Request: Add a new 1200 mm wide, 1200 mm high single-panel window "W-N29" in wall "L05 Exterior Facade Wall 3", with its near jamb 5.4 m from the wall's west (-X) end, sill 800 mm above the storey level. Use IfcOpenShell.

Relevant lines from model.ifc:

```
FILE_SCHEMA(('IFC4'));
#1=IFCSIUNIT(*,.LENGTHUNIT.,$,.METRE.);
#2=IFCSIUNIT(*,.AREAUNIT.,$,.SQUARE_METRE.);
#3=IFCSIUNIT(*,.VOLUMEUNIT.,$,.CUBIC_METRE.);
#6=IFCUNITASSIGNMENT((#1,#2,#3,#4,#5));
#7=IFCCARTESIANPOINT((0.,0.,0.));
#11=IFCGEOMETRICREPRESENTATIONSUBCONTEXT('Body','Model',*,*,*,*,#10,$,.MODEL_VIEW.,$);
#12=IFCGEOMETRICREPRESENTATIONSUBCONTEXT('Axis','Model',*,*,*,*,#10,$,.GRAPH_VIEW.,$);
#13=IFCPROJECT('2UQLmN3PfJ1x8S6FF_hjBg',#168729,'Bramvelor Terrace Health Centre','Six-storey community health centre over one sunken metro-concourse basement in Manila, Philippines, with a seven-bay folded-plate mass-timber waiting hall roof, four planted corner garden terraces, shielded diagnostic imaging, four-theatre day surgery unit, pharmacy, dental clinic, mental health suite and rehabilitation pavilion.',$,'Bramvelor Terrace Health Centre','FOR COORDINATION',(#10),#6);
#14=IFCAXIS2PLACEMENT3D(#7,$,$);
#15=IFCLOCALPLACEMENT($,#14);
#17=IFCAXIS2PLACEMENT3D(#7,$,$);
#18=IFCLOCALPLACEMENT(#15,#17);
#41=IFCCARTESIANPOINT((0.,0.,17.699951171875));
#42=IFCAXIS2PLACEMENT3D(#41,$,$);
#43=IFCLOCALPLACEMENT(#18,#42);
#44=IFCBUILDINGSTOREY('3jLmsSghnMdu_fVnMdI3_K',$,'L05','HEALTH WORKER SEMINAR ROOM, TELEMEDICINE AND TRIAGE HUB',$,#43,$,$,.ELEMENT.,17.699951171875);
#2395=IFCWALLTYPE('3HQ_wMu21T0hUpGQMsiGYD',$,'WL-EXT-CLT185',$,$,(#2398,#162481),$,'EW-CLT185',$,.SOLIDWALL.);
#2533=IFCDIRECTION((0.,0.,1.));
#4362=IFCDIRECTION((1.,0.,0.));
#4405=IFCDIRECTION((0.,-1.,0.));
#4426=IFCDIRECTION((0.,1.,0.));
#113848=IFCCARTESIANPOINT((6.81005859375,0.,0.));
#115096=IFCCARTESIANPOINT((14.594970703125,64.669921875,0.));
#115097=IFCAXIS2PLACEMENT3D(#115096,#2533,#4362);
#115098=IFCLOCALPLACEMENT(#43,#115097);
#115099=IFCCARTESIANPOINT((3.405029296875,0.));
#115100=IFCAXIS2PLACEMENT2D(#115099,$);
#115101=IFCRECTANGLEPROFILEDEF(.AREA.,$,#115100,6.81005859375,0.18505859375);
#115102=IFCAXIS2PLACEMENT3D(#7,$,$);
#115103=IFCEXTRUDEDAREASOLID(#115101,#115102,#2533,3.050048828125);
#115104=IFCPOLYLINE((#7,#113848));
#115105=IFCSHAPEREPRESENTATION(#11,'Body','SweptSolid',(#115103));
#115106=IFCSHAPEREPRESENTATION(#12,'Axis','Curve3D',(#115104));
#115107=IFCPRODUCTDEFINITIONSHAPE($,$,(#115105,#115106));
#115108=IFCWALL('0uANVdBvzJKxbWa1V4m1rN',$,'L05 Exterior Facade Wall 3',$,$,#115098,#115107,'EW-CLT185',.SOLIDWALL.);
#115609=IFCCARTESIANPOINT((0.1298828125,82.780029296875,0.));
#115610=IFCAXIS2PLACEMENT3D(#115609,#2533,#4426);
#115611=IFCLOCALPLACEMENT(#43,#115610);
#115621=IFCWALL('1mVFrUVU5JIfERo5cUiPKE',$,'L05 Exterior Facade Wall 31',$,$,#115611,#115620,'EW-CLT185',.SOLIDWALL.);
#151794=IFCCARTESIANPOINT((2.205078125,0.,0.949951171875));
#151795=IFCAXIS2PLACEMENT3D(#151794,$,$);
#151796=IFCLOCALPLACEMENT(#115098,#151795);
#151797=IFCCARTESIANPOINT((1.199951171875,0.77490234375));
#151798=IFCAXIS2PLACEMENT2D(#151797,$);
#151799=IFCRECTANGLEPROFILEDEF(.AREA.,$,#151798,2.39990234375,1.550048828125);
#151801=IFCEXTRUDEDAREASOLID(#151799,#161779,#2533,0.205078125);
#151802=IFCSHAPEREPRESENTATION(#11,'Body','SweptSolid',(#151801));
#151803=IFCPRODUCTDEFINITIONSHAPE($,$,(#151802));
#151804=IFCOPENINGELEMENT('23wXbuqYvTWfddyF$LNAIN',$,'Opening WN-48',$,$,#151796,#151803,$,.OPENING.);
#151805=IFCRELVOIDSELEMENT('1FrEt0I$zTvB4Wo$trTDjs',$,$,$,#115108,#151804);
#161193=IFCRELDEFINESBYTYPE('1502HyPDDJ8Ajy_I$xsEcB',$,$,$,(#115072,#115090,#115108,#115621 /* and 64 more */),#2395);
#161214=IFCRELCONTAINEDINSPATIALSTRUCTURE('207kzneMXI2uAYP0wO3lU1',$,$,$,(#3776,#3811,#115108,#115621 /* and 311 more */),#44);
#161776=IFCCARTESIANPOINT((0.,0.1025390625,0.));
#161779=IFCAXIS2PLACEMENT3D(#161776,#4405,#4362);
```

```python
import numpy as np
import ifcopenshell
import ifcopenshell.api.feature
import ifcopenshell.api.geometry
import ifcopenshell.api.root
import ifcopenshell.api.spatial
import ifcopenshell.geom
import ifcopenshell.util.element
import ifcopenshell.util.placement
import ifcopenshell.util.representation
import ifcopenshell.util.shape
import ifcopenshell.util.unit

model = ifcopenshell.open("model.ifc")
unit_scale = ifcopenshell.util.unit.calculate_unit_scale(model)
settings = ifcopenshell.geom.settings()


def volume(element):
    """Net volume in cubic metres, openings subtracted."""
    shape = ifcopenshell.geom.create_shape(settings, element)
    return ifcopenshell.util.shape.get_volume(shape.geometry)


wall = model.by_guid("0uANVdBvzJKxbWa1V4m1rN")
storey = ifcopenshell.util.element.get_container(wall, ifc_class="IfcBuildingStorey")
context = ifcopenshell.util.representation.get_context(model, "Model", "Body", "MODEL_VIEW")
before = volume(wall)

width, height, from_end, sill = 1.2, 1.2, 5.4, 0.8  # metres

# The wall runs along its own X axis, and the end named is its -X end.
wall_shape = ifcopenshell.geom.create_shape(settings, wall)
x, y, z = ifcopenshell.util.shape.get_vertices(wall_shape.geometry).T
start = x.min() + from_end
face, thickness = float(y.min()), float(y.max() - y.min())
wall_matrix = ifcopenshell.util.placement.get_local_placement(wall.ObjectPlacement)
level = ifcopenshell.util.placement.get_local_placement(storey.ObjectPlacement)[2, 3]


def in_wall(x, y):
    """Placement at x, y metres in the wall's axes, at sill height."""
    matrix = wall_matrix.copy()
    matrix[:, 3] = wall_matrix @ np.array([x / unit_scale, y / unit_scale, 0.0, 1.0])
    matrix[2, 3] = level + sill / unit_scale
    return matrix


# Opening: a box that overshoots both wall faces by 50 mm.
opening = ifcopenshell.api.root.create_entity(model, ifc_class="IfcOpeningElement", predefined_type="OPENING")
box = ifcopenshell.api.geometry.add_wall_representation(
    model, context=context, length=width, height=height, thickness=thickness + 0.1
)
ifcopenshell.api.geometry.assign_representation(model, product=opening, representation=box)
ifcopenshell.api.geometry.edit_object_placement(model, product=opening, matrix=in_wall(start, face - 0.05), is_si=False)
ifcopenshell.api.feature.add_feature(model, feature=opening, element=wall)

window = ifcopenshell.api.root.create_entity(model, ifc_class="IfcWindow", name="W-N29", predefined_type="WINDOW")
window.OverallWidth, window.OverallHeight = width / unit_scale, height / unit_scale
window.PartitioningType = "SINGLE_PANEL"
body = ifcopenshell.api.geometry.add_window_representation(
    model,
    context=context,
    overall_width=window.OverallWidth,
    overall_height=window.OverallHeight,
    partition_type="SINGLE_PANEL",
)
ifcopenshell.api.geometry.assign_representation(model, product=window, representation=body)
ifcopenshell.api.spatial.assign_container(model, products=[window], relating_structure=storey)
ifcopenshell.api.feature.add_filling(model, opening=opening, element=window)

# Centre the window in the wall's thickness.
ifcopenshell.api.geometry.edit_object_placement(model, product=window, matrix=in_wall(start, face), is_si=False)
window_shape = ifcopenshell.geom.create_shape(settings, window)
depth = ifcopenshell.util.shape.get_vertices(window_shape.geometry)[:, 1]
offset = face + thickness / 2 - (depth.min() + depth.max()) / 2
ifcopenshell.api.geometry.edit_object_placement(model, product=window, matrix=in_wall(start, offset), is_si=False)

after = volume(wall)

print(f"wall volume {before:.3f} -> {after:.3f} m3")

model.write("model_updated.ifc")
```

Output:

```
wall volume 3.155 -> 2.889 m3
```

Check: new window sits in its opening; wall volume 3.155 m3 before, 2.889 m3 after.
